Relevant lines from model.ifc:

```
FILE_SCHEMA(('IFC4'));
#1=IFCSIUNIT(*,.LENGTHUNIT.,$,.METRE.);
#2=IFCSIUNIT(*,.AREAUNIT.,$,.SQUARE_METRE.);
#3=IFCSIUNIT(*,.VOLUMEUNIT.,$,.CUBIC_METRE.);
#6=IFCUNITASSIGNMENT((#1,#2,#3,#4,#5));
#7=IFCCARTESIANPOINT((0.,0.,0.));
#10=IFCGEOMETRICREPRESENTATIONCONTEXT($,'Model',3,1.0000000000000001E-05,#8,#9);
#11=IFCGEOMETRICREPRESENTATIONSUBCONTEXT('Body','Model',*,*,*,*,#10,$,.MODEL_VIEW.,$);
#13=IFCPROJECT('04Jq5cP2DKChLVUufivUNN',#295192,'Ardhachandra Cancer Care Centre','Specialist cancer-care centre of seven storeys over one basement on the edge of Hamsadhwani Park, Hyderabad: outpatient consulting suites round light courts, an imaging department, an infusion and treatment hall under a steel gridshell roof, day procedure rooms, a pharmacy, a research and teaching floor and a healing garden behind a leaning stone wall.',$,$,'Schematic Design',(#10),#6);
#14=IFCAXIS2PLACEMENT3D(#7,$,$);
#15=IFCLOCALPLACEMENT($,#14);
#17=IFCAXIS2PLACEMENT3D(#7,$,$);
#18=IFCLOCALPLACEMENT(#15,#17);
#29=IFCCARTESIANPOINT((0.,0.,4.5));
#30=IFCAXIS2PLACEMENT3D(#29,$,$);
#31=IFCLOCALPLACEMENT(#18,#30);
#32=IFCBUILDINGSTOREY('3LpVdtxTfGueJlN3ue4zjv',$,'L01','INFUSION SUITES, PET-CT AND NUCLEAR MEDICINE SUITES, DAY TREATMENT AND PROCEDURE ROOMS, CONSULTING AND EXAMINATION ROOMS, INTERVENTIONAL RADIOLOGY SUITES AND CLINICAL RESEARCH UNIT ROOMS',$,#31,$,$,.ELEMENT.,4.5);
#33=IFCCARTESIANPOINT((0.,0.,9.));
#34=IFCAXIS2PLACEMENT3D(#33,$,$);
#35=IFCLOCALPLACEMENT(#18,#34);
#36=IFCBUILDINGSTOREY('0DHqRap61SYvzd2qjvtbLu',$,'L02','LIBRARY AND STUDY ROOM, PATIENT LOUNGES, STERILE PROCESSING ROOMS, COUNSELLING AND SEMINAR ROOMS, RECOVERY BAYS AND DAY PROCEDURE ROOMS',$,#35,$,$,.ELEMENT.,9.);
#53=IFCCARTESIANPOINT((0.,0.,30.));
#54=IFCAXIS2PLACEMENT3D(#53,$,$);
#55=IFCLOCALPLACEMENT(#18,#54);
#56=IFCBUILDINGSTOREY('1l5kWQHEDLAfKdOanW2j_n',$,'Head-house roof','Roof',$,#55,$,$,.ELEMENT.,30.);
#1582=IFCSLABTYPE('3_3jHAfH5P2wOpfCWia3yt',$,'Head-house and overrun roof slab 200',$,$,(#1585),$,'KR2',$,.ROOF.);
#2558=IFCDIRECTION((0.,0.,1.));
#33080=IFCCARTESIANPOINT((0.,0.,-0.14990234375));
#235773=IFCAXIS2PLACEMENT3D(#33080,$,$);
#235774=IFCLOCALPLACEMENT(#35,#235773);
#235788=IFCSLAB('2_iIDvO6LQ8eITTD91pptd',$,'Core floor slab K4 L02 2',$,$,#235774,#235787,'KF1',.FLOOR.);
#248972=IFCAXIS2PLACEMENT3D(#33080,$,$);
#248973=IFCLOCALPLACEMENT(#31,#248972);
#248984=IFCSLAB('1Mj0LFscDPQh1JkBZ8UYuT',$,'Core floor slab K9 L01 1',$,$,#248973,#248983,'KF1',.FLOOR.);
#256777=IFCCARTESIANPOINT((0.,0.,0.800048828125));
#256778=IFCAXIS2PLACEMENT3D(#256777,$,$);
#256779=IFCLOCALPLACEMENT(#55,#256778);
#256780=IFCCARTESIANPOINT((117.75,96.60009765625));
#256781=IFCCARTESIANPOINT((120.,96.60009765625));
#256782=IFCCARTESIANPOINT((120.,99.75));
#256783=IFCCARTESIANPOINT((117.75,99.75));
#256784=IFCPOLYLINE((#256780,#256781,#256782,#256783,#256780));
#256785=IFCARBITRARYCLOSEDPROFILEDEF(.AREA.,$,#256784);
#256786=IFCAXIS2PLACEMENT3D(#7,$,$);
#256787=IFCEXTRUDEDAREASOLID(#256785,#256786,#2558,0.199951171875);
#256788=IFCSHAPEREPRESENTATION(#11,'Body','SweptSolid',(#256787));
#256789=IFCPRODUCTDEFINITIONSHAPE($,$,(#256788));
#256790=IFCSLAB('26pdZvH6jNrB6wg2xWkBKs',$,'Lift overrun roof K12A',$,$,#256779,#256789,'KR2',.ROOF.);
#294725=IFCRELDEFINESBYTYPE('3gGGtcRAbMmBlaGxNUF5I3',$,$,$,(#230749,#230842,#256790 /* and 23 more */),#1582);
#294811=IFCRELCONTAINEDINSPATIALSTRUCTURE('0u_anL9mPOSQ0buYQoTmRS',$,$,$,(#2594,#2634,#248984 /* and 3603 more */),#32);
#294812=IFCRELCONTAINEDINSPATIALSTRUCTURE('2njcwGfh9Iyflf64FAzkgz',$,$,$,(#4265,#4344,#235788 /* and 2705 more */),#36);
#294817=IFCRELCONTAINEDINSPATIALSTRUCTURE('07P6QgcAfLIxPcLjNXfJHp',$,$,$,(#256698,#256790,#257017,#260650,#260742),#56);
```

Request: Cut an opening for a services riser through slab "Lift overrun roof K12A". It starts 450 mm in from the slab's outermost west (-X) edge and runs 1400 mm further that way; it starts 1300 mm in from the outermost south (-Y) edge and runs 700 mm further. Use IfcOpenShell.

```python
import numpy as np
import ifcopenshell
import ifcopenshell.api.feature
import ifcopenshell.api.geometry
import ifcopenshell.api.root
import ifcopenshell.geom
import ifcopenshell.util.placement
import ifcopenshell.util.representation
import ifcopenshell.util.shape
import ifcopenshell.util.unit

model = ifcopenshell.open("model.ifc")
unit_scale = ifcopenshell.util.unit.calculate_unit_scale(model)
settings = ifcopenshell.geom.settings()


def volume(element):
    """Net volume in cubic metres, openings subtracted."""
    shape = ifcopenshell.geom.create_shape(settings, element)
    return ifcopenshell.util.shape.get_volume(shape.geometry)


slab = model.by_id(256790)
before = volume(slab)

# Extent in the slab's own axes, in metres. The edges named are its -X and -Y sides.
slab_shape = ifcopenshell.geom.create_shape(settings, slab)
vertices = ifcopenshell.util.shape.get_vertices(slab_shape.geometry)
x_min, y_min, bottom = vertices.min(axis=0)
top = vertices[:, 2].max()

opening = ifcopenshell.api.root.create_entity(model, ifc_class="IfcOpeningElement", name="Services riser opening", predefined_type="OPENING")
context = ifcopenshell.util.representation.get_context(model, "Model", "Body", "MODEL_VIEW")
width, depth = 1.4, 0.7
outline = [(0.0, 0.0), (width, 0.0), (width, depth), (0.0, depth), (0.0, 0.0)]
# Overshoot both faces by 50 mm so the cut is clean.
shape = ifcopenshell.api.geometry.add_slab_representation(
    model, context=context, depth=top - bottom + 0.1, polyline=outline
)
ifcopenshell.api.geometry.assign_representation(model, product=opening, representation=shape)

matrix = ifcopenshell.util.placement.get_local_placement(slab.ObjectPlacement)
matrix[:, 3] = matrix @ np.append(np.array([x_min + 0.45, y_min + 1.3, bottom - 0.05]) / unit_scale, 1.0)
ifcopenshell.api.geometry.edit_object_placement(model, product=opening, matrix=matrix, is_si=False)
ifcopenshell.api.feature.add_feature(model, feature=opening, element=slab)

after = volume(slab)

print(f"slab volume {before:.3f} -> {after:.3f} m3")

model.write("model_v2.ifc")
```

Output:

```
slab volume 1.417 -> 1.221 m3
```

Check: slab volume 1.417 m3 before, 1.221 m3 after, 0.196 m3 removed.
